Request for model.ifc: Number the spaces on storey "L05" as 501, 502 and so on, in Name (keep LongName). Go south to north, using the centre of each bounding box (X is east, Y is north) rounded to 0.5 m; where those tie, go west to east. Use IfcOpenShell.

First a look at what the model holds.

```python
import ifcopenshell
import ifcopenshell.util.element
import ifcopenshell.util.placement

model = ifcopenshell.open("model.ifc")
print(model.schema)
storey = next(s for s in model.by_type("IfcBuildingStorey") if s.Name == "L05")
spaces = [e for e in ifcopenshell.util.element.get_decomposition(storey) if e.is_a("IfcSpace")]
for e in sorted(spaces, key=lambda e: e.id()):
    origin = ifcopenshell.util.placement.get_local_placement(e.ObjectPlacement)[:3, 3]
    print(e.id(), e.Name, e.LongName, origin.round(2) + 0.0, sep=" | ")
```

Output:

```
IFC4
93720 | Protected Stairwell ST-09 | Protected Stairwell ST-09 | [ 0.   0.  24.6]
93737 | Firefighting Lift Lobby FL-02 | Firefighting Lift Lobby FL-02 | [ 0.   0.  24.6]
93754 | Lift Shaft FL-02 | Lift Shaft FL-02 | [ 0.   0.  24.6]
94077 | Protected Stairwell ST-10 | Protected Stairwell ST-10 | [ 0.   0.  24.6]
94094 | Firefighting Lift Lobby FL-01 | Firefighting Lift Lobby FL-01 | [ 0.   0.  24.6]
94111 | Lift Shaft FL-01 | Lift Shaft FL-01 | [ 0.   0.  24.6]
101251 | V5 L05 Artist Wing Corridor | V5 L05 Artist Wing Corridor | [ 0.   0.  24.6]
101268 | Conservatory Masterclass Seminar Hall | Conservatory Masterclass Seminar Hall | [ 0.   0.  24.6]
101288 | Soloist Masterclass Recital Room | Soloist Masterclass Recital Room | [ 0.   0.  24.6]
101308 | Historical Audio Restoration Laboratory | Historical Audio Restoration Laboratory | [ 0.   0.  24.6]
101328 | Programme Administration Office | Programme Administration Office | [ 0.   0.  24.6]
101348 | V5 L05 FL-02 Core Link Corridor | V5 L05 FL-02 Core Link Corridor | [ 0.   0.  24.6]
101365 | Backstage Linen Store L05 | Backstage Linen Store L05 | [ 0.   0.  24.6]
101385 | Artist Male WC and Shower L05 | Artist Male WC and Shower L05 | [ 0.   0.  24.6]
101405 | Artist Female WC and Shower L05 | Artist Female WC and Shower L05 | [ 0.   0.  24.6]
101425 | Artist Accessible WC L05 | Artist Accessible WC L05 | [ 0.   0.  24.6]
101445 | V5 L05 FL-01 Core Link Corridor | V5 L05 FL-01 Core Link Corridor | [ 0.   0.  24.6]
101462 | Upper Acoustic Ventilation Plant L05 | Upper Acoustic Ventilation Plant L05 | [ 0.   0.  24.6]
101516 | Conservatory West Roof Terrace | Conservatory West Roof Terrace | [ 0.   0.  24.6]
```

```python
import ifcopenshell
import ifcopenshell.geom
import ifcopenshell.util.element
import ifcopenshell.util.shape

model = ifcopenshell.open("model.ifc")
settings = ifcopenshell.geom.settings()
settings.set("use-world-coords", True)


def centre(element):
    shape = ifcopenshell.geom.create_shape(settings, element)
    return ifcopenshell.util.shape.get_bbox_centroid(shape.geometry)


storey = next(s for s in model.by_type("IfcBuildingStorey") if s.Name == "L05")
spaces = [e for e in ifcopenshell.util.element.get_decomposition(storey) if e.is_a("IfcSpace")]

# Insertion points can sit at a corner or the storey origin, so sort by the geometry (in metres).
centres = {e: centre(e) for e in spaces}
spaces.sort(key=lambda e: (round(centres[e][1] / 0.5), centres[e][0]))

for i, e in enumerate(spaces, start=1):
    number = f"5{i:02d}"
    e.Name = number
    print(e.id(), number)

model.write("model-out.ifc")
```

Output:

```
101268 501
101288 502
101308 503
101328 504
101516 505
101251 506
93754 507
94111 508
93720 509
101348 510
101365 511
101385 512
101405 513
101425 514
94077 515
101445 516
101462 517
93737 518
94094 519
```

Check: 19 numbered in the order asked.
